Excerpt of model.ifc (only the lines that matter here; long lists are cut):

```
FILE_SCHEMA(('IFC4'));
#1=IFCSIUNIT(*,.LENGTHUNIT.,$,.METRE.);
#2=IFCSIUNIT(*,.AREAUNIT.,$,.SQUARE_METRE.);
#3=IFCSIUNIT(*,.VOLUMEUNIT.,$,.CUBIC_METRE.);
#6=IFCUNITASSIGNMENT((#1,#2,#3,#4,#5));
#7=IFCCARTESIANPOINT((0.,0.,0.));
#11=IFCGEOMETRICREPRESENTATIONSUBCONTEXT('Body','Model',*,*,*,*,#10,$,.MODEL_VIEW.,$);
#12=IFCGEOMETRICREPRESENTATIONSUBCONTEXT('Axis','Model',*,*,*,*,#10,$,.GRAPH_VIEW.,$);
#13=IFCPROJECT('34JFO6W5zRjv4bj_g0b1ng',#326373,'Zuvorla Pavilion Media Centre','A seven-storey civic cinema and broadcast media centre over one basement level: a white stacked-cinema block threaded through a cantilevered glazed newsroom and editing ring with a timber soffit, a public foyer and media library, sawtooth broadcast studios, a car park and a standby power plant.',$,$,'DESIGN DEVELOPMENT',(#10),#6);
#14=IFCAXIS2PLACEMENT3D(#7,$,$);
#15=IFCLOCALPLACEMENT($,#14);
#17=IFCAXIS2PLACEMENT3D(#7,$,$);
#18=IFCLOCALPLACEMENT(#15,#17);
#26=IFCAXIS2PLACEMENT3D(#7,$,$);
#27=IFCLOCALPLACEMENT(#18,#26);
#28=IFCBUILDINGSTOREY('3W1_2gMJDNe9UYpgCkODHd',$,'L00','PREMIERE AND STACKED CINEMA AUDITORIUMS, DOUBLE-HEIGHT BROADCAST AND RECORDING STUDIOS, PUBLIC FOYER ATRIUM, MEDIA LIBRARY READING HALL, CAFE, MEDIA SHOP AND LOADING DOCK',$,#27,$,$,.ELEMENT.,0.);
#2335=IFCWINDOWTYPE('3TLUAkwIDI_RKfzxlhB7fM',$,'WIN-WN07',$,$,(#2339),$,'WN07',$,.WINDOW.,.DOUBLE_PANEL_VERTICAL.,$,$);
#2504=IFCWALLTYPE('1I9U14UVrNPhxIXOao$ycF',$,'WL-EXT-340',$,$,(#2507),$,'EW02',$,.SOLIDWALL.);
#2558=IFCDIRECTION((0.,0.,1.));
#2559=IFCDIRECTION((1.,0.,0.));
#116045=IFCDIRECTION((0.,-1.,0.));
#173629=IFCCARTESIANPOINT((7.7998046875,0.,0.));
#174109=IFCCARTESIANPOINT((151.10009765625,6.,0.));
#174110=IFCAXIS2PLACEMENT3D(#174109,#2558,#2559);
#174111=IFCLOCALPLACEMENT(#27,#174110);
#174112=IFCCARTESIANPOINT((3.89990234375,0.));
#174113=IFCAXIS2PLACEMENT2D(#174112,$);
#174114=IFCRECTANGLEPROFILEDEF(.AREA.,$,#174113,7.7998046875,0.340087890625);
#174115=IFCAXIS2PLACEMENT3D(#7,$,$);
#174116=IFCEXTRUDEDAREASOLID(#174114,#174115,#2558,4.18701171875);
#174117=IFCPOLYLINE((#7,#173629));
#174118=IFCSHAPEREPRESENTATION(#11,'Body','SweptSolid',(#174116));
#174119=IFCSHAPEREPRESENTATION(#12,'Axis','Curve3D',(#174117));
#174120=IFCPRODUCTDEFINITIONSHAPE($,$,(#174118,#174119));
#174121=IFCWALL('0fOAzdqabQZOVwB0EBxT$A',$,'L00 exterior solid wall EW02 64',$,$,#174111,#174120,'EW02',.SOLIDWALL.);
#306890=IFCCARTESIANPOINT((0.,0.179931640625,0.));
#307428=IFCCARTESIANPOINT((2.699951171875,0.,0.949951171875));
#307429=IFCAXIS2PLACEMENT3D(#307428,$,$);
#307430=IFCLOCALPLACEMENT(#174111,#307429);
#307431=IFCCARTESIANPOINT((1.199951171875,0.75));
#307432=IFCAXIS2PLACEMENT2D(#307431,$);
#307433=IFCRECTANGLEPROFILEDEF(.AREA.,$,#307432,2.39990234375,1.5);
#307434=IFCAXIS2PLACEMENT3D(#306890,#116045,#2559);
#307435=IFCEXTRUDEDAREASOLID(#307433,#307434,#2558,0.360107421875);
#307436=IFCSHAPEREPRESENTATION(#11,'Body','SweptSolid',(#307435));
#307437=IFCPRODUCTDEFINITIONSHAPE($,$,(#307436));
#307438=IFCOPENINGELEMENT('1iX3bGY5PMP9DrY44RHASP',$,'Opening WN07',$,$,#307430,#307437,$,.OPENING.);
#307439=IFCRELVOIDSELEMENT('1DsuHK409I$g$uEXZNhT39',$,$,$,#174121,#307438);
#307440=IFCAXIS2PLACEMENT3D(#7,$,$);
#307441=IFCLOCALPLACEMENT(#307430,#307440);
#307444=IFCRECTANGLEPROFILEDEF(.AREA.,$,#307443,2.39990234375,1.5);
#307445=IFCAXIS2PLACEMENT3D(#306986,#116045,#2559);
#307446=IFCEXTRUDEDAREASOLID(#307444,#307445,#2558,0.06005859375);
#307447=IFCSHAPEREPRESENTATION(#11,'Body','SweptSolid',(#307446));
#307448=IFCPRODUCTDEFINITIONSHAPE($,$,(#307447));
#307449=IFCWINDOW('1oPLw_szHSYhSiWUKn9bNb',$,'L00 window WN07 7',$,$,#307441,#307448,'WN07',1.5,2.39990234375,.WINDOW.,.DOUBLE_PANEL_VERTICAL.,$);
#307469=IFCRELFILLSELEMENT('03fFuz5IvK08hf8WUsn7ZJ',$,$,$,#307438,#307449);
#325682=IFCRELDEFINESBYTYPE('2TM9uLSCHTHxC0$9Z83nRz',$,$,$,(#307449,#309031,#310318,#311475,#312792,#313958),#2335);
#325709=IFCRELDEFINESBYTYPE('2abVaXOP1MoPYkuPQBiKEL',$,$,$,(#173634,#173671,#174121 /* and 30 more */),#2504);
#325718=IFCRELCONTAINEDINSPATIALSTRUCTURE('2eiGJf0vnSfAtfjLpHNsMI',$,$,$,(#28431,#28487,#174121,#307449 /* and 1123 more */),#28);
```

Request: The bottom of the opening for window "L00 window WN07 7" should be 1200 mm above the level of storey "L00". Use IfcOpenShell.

```python
import numpy as np
import ifcopenshell
import ifcopenshell.api.geometry
import ifcopenshell.geom
import ifcopenshell.util.element
import ifcopenshell.util.placement
import ifcopenshell.util.shape
import ifcopenshell.util.unit

model = ifcopenshell.open("model.ifc")
unit_scale = ifcopenshell.util.unit.calculate_unit_scale(model)

window = model.by_id(307449)
opening = window.FillsVoids[0].RelatingOpeningElement
storey = ifcopenshell.util.element.get_container(window, ifc_class="IfcBuildingStorey")
level = ifcopenshell.util.placement.get_local_placement(storey.ObjectPlacement)[2, 3]

# The opening's origin need not be at the sill, so measure its lowest point.
shape = ifcopenshell.geom.create_shape(ifcopenshell.geom.settings(), opening)
bottom = ifcopenshell.util.shape.get_shape_bottom_elevation(shape, shape.geometry) / unit_scale
dz = level + 1.2 - bottom

shift = np.array([0.0, 0.0, dz])
# The window is placed relative to its opening, so it follows when the opening moves.
matrix = ifcopenshell.util.placement.get_local_placement(opening.ObjectPlacement)
matrix[:3, 3] += shift
ifcopenshell.api.geometry.edit_object_placement(
    model, product=opening, matrix=matrix, is_si=False, should_transform_children=True
)

print(f"moved by {dz * unit_scale:+.3f} m")

model.write("model-out.ifc")
```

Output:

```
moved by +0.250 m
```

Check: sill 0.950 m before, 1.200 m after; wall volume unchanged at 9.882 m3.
